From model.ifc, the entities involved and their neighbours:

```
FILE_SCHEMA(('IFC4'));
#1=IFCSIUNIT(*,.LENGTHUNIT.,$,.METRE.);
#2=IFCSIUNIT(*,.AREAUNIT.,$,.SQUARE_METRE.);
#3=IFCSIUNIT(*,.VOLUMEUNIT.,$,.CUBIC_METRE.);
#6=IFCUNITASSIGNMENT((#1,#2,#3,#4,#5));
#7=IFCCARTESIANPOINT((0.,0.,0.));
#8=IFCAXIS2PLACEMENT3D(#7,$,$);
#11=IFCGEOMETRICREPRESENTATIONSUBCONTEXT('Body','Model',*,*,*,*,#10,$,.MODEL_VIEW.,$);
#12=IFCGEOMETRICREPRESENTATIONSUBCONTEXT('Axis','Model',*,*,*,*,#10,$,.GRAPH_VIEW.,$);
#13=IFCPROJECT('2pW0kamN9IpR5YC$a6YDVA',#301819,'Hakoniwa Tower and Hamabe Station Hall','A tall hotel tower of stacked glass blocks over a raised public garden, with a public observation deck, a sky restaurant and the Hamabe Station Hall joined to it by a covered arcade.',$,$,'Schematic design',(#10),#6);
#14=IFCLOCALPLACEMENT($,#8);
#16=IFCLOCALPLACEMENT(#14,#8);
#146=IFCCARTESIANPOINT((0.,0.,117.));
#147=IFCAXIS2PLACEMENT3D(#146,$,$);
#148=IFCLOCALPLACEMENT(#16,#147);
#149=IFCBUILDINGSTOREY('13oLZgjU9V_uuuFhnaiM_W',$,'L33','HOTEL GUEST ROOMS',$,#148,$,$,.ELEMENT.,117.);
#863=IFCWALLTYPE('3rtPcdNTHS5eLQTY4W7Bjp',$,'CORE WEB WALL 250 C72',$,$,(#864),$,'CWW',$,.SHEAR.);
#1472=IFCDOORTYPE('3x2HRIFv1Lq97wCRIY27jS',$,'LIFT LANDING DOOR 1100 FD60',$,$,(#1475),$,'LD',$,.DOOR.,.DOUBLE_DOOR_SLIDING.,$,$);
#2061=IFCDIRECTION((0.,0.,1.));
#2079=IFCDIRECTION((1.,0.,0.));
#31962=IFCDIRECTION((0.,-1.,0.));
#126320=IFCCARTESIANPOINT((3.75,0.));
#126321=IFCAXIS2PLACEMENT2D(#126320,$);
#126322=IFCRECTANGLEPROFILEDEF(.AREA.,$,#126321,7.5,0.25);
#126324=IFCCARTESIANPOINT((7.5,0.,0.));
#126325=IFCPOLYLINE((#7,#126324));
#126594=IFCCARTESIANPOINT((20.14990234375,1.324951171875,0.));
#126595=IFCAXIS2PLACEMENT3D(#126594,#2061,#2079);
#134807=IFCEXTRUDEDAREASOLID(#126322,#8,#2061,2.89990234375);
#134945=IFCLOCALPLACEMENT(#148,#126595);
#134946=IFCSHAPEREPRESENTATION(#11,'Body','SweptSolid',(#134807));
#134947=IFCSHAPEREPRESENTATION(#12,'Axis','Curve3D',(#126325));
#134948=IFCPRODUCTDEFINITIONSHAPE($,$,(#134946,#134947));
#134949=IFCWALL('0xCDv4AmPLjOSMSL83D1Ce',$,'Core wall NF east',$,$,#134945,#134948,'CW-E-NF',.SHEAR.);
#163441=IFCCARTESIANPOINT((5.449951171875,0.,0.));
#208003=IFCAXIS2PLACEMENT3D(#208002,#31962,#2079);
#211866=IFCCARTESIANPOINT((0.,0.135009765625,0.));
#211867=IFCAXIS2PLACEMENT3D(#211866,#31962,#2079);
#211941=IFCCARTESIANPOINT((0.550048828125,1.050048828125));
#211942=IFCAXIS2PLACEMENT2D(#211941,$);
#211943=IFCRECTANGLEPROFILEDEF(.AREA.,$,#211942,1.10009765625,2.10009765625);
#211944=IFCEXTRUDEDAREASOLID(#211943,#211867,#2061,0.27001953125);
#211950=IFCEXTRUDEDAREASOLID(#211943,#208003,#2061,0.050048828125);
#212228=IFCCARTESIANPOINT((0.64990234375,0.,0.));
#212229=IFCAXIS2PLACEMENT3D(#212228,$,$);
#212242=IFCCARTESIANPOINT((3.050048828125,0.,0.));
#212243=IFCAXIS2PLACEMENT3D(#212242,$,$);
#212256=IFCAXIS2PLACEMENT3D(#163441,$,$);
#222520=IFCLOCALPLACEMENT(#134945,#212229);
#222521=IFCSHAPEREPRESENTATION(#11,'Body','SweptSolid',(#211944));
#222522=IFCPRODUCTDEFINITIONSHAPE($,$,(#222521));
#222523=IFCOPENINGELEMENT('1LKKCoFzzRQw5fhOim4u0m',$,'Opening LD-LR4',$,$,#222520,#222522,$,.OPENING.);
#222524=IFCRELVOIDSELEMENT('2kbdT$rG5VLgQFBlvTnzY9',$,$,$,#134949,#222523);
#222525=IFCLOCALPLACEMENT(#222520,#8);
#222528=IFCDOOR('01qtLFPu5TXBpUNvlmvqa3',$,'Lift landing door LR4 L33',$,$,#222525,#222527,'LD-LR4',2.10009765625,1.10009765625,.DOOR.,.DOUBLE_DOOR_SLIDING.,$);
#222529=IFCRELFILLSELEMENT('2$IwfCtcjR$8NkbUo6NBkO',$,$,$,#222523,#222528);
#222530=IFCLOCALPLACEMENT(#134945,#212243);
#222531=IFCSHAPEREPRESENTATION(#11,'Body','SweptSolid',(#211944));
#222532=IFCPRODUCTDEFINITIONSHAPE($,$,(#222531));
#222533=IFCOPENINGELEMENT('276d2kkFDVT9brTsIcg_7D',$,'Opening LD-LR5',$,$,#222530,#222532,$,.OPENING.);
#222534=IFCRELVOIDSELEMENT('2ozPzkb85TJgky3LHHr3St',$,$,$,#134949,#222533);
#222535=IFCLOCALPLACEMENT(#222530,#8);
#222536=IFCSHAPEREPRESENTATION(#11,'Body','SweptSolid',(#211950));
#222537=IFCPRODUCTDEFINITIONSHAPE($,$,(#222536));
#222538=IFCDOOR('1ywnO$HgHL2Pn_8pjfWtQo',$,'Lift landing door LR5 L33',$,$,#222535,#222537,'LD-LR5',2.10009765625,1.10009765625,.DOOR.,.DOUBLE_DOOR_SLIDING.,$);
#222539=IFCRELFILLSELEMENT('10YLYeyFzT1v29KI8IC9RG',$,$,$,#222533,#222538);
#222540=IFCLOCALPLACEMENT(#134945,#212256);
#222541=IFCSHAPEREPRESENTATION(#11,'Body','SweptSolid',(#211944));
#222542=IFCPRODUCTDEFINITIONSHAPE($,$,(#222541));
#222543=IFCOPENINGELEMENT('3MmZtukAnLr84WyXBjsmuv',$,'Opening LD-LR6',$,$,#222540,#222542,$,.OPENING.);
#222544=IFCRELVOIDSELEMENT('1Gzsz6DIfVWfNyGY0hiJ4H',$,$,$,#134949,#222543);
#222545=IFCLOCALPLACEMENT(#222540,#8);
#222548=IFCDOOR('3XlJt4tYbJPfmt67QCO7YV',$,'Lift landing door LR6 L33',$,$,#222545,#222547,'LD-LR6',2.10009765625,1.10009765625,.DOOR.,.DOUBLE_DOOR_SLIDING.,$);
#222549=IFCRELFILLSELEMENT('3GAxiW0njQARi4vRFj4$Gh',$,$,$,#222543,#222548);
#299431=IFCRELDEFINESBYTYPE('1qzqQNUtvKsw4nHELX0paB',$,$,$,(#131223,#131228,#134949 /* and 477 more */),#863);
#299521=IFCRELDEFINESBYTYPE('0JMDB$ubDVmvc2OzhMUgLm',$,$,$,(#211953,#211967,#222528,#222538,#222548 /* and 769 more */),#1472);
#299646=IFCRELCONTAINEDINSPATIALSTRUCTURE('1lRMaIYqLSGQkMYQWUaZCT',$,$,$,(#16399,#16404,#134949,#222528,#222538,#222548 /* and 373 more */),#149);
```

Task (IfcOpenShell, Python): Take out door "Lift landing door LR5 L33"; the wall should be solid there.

```python
import ifcopenshell
import ifcopenshell.api.feature
import ifcopenshell.api.root
import ifcopenshell.geom
import ifcopenshell.util.shape

model = ifcopenshell.open("model.ifc")
settings = ifcopenshell.geom.settings()


def volume(element):
    """Net volume in cubic metres, openings subtracted."""
    shape = ifcopenshell.geom.create_shape(settings, element)
    return ifcopenshell.util.shape.get_volume(shape.geometry)


door = model.by_guid("1ywnO$HgHL2Pn_8pjfWtQo")
opening = door.FillsVoids[0].RelatingOpeningElement
wall = opening.VoidsElements[0].RelatingBuildingElement
before = volume(wall)

ifcopenshell.api.root.remove_product(model, product=door)
ifcopenshell.api.feature.remove_feature(model, feature=opening)

after = volume(wall)

print(f"wall volume {before:.3f} -> {after:.3f} m3")

model.write("model_v2.ifc")
```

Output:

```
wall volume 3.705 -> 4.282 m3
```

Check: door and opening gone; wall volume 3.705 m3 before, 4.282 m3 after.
